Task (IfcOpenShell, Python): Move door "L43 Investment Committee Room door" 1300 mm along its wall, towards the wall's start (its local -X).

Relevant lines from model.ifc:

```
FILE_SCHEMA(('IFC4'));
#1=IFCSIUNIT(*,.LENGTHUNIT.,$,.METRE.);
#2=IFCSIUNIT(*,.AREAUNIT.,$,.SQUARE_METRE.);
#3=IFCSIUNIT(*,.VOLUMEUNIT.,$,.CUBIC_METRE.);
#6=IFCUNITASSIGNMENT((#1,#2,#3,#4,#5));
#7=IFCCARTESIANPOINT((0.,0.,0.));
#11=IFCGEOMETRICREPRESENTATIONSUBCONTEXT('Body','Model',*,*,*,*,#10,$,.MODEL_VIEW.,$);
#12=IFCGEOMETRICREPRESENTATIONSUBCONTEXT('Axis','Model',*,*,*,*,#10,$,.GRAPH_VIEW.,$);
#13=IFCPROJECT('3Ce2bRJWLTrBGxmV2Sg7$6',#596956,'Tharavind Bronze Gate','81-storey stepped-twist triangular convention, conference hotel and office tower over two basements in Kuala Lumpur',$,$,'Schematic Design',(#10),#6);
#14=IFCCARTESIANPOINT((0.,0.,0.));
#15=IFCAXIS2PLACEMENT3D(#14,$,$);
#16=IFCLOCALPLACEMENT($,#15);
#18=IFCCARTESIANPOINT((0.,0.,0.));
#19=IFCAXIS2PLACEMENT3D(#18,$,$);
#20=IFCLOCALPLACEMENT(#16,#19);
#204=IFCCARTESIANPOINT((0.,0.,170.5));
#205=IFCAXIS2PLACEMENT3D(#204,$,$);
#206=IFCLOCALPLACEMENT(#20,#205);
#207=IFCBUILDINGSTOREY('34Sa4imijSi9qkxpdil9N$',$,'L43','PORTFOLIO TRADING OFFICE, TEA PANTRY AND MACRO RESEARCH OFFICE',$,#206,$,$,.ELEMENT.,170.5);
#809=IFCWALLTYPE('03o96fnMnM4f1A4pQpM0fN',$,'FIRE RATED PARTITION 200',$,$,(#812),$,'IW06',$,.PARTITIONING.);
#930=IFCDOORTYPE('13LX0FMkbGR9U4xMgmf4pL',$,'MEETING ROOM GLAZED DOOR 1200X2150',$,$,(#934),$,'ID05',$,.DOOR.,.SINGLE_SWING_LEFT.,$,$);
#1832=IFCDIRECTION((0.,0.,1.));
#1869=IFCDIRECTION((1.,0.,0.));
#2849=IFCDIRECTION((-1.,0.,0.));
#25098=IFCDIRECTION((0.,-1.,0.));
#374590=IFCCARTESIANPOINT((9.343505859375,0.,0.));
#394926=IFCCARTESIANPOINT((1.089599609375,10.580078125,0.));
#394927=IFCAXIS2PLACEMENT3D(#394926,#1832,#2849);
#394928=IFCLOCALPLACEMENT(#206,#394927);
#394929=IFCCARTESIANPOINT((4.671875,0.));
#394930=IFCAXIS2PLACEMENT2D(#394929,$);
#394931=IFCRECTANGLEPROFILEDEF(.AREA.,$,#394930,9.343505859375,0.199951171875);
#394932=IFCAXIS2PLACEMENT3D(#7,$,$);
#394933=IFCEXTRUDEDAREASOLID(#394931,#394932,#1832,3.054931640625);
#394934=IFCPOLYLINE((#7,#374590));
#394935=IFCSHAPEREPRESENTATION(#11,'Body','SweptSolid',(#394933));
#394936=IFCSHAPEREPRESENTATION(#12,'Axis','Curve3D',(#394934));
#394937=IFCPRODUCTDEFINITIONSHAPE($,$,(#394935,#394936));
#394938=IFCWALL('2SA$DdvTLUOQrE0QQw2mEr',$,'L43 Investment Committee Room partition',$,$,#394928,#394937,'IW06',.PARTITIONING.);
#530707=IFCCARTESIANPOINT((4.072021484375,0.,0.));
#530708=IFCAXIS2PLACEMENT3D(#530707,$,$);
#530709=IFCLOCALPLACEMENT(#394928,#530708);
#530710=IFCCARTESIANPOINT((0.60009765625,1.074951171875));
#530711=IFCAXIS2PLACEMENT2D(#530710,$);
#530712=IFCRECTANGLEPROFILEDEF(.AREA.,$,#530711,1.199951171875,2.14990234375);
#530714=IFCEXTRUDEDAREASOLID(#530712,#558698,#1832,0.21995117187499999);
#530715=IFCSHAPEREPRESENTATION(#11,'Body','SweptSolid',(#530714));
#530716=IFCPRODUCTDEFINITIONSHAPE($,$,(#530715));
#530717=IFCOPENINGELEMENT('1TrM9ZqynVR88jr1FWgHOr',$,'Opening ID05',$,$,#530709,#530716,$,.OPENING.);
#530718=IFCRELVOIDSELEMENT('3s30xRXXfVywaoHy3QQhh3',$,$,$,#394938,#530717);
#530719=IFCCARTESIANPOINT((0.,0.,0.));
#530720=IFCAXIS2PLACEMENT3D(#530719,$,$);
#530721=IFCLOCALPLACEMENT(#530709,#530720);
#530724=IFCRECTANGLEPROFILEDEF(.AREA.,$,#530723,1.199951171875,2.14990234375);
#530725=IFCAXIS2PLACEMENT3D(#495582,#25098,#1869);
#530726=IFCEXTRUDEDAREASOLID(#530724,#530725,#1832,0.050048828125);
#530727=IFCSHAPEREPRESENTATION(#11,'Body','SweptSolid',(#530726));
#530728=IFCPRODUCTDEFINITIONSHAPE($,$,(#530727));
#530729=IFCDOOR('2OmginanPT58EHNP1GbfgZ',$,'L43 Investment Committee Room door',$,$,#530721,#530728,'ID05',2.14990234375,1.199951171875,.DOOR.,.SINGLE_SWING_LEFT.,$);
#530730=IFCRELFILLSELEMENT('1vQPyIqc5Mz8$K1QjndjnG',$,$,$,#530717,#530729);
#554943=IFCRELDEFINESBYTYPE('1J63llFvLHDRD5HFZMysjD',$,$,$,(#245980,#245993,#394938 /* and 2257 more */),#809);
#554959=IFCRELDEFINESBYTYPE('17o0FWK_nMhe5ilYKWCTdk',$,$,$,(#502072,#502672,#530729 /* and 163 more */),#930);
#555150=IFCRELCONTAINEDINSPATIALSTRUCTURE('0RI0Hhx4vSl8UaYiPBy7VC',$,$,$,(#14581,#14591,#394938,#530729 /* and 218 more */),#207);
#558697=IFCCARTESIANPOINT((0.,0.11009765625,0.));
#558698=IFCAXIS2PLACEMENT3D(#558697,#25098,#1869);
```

```python
import ifcopenshell
import ifcopenshell.api.geometry
import ifcopenshell.util.placement
import ifcopenshell.util.unit

model = ifcopenshell.open("model.ifc")
unit_scale = ifcopenshell.util.unit.calculate_unit_scale(model)

door = model.by_id(530729)
opening = door.FillsVoids[0].RelatingOpeningElement
wall = opening.VoidsElements[0].RelatingBuildingElement

wall_matrix = ifcopenshell.util.placement.get_local_placement(wall.ObjectPlacement)
shift = wall_matrix[:3, 0] * -1.3 / unit_scale
before = ifcopenshell.util.placement.get_local_placement(door.ObjectPlacement)[:3, 3].copy()

# The door is placed relative to its opening, so it follows when the opening moves.
matrix = ifcopenshell.util.placement.get_local_placement(opening.ObjectPlacement)
matrix[:3, 3] += shift
ifcopenshell.api.geometry.edit_object_placement(
    model, product=opening, matrix=matrix, is_si=False, should_transform_children=True
)

after = ifcopenshell.util.placement.get_local_placement(door.ObjectPlacement)[:3, 3]
print("door moved by", (after - before).round(3) + 0.0)

model.write("model_updated.ifc")
```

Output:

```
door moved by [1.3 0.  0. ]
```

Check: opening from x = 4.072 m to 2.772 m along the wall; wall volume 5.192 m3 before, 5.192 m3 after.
